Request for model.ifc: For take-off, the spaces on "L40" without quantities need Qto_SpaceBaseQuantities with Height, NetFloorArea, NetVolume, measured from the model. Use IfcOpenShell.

First a look at what the model holds.

```python
import ifcopenshell
import ifcopenshell.util.element
import ifcopenshell.util.unit

model = ifcopenshell.open("model.ifc")
print(model.schema)
for unit_type in ("LENGTHUNIT", "AREAUNIT", "VOLUMEUNIT"):
    print(unit_type, ifcopenshell.util.unit.calculate_unit_scale(model, unit_type))
storey = next(s for s in model.by_type("IfcBuildingStorey") if s.Name == "L40")
spaces = [e for e in ifcopenshell.util.element.get_decomposition(storey) if e.is_a("IfcSpace")]
for e in sorted(spaces, key=lambda e: e.id()):
    print(e.id(), e.is_a(), e.Name, list(ifcopenshell.util.element.get_psets(e, qtos_only=True)), sep=" | ")
```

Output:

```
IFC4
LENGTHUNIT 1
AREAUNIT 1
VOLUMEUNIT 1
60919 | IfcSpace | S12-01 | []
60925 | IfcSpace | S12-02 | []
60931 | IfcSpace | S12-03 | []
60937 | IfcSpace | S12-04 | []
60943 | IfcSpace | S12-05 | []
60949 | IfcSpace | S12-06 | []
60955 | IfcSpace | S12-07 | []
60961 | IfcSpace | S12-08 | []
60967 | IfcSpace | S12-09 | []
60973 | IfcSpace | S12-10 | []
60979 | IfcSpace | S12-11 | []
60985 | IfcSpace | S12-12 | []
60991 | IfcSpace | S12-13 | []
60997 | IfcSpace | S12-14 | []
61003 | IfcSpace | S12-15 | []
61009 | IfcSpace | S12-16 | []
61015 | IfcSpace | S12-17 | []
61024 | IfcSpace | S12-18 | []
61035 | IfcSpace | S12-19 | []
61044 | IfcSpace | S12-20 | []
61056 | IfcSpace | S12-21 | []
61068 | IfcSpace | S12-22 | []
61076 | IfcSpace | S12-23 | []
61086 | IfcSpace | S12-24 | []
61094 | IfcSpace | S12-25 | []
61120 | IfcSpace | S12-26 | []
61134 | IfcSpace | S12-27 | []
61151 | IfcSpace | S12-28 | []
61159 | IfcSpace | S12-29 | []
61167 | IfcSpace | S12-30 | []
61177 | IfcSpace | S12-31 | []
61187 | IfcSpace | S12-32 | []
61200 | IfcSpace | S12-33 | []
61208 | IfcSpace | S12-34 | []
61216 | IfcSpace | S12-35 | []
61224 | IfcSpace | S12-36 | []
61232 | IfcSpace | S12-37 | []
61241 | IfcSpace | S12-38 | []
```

```python
import ifcopenshell
import ifcopenshell.api.pset
import ifcopenshell.geom
import ifcopenshell.util.element
import ifcopenshell.util.shape
import ifcopenshell.util.unit

model = ifcopenshell.open("model.ifc")
unit_scale = ifcopenshell.util.unit.calculate_unit_scale(model)
area_scale = ifcopenshell.util.unit.calculate_unit_scale(model, "AREAUNIT")
volume_scale = ifcopenshell.util.unit.calculate_unit_scale(model, "VOLUMEUNIT")
settings = ifcopenshell.geom.settings()

storey = next(s for s in model.by_type("IfcBuildingStorey") if s.Name == "L40")
spaces = [e for e in ifcopenshell.util.element.get_decomposition(storey) if e.is_a("IfcSpace")]

for e in sorted(spaces, key=lambda e: e.id()):
    if ifcopenshell.util.element.get_psets(e, qtos_only=True, should_inherit=False):
        continue
    # Geometry comes back in metres, in the element's own axes.
    shape = ifcopenshell.geom.create_shape(settings, e)
    values = {
        "Height": ifcopenshell.util.shape.get_z(shape.geometry) / unit_scale,
        "NetFloorArea": ifcopenshell.util.shape.get_footprint_area(shape.geometry) / area_scale,
        "NetVolume": ifcopenshell.util.shape.get_volume(shape.geometry) / volume_scale,
    }
    qto = ifcopenshell.api.pset.add_qto(model, product=e, name="Qto_SpaceBaseQuantities")
    ifcopenshell.api.pset.edit_qto(model, qto=qto, properties=values)
    print(e.id(), {k: round(v, 3) for k, v in values.items()})

model.write("model-out.ifc")
```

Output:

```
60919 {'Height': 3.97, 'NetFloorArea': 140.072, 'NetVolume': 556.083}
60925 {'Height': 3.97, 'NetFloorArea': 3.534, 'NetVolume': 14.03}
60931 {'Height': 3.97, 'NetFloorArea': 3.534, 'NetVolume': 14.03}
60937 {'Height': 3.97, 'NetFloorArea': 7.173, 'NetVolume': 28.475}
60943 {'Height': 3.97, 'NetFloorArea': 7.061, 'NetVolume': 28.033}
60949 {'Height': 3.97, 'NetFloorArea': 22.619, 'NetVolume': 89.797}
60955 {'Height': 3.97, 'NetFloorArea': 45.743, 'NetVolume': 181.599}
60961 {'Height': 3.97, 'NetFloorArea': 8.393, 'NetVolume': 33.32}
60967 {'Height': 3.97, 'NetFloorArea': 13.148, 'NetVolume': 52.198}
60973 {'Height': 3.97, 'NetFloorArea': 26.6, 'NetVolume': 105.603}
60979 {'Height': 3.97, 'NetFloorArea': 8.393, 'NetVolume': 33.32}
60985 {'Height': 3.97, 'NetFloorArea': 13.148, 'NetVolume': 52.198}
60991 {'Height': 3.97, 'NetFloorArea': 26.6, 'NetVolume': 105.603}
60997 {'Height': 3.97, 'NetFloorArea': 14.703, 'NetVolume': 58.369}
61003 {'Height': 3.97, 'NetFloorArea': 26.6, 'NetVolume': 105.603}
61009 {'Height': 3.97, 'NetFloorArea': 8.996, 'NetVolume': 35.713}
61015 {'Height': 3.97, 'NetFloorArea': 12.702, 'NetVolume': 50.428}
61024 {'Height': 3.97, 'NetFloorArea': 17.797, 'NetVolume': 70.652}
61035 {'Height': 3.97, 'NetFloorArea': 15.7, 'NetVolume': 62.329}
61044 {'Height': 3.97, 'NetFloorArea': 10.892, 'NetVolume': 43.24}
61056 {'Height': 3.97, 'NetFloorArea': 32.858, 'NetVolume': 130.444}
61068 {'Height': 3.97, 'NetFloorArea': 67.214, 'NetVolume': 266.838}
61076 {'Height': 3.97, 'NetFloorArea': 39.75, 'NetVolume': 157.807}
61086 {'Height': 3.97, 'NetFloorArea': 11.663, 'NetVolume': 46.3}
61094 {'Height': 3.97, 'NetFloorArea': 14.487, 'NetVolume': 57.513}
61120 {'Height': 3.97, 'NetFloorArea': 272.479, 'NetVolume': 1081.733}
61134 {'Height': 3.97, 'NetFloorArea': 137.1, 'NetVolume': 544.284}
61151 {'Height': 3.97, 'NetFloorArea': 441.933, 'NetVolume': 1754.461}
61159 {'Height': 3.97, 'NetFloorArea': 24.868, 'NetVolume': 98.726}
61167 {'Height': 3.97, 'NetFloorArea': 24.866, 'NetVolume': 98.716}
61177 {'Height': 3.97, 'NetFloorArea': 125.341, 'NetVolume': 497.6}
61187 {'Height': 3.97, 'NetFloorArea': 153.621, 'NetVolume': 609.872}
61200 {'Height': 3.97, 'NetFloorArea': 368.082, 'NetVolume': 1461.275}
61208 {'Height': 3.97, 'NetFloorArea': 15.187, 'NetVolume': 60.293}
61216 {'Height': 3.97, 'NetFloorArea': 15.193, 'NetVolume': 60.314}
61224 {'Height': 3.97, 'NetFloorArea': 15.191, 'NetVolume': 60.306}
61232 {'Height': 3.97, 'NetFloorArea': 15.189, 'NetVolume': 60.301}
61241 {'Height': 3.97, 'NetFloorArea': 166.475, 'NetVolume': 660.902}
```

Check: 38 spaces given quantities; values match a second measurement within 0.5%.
